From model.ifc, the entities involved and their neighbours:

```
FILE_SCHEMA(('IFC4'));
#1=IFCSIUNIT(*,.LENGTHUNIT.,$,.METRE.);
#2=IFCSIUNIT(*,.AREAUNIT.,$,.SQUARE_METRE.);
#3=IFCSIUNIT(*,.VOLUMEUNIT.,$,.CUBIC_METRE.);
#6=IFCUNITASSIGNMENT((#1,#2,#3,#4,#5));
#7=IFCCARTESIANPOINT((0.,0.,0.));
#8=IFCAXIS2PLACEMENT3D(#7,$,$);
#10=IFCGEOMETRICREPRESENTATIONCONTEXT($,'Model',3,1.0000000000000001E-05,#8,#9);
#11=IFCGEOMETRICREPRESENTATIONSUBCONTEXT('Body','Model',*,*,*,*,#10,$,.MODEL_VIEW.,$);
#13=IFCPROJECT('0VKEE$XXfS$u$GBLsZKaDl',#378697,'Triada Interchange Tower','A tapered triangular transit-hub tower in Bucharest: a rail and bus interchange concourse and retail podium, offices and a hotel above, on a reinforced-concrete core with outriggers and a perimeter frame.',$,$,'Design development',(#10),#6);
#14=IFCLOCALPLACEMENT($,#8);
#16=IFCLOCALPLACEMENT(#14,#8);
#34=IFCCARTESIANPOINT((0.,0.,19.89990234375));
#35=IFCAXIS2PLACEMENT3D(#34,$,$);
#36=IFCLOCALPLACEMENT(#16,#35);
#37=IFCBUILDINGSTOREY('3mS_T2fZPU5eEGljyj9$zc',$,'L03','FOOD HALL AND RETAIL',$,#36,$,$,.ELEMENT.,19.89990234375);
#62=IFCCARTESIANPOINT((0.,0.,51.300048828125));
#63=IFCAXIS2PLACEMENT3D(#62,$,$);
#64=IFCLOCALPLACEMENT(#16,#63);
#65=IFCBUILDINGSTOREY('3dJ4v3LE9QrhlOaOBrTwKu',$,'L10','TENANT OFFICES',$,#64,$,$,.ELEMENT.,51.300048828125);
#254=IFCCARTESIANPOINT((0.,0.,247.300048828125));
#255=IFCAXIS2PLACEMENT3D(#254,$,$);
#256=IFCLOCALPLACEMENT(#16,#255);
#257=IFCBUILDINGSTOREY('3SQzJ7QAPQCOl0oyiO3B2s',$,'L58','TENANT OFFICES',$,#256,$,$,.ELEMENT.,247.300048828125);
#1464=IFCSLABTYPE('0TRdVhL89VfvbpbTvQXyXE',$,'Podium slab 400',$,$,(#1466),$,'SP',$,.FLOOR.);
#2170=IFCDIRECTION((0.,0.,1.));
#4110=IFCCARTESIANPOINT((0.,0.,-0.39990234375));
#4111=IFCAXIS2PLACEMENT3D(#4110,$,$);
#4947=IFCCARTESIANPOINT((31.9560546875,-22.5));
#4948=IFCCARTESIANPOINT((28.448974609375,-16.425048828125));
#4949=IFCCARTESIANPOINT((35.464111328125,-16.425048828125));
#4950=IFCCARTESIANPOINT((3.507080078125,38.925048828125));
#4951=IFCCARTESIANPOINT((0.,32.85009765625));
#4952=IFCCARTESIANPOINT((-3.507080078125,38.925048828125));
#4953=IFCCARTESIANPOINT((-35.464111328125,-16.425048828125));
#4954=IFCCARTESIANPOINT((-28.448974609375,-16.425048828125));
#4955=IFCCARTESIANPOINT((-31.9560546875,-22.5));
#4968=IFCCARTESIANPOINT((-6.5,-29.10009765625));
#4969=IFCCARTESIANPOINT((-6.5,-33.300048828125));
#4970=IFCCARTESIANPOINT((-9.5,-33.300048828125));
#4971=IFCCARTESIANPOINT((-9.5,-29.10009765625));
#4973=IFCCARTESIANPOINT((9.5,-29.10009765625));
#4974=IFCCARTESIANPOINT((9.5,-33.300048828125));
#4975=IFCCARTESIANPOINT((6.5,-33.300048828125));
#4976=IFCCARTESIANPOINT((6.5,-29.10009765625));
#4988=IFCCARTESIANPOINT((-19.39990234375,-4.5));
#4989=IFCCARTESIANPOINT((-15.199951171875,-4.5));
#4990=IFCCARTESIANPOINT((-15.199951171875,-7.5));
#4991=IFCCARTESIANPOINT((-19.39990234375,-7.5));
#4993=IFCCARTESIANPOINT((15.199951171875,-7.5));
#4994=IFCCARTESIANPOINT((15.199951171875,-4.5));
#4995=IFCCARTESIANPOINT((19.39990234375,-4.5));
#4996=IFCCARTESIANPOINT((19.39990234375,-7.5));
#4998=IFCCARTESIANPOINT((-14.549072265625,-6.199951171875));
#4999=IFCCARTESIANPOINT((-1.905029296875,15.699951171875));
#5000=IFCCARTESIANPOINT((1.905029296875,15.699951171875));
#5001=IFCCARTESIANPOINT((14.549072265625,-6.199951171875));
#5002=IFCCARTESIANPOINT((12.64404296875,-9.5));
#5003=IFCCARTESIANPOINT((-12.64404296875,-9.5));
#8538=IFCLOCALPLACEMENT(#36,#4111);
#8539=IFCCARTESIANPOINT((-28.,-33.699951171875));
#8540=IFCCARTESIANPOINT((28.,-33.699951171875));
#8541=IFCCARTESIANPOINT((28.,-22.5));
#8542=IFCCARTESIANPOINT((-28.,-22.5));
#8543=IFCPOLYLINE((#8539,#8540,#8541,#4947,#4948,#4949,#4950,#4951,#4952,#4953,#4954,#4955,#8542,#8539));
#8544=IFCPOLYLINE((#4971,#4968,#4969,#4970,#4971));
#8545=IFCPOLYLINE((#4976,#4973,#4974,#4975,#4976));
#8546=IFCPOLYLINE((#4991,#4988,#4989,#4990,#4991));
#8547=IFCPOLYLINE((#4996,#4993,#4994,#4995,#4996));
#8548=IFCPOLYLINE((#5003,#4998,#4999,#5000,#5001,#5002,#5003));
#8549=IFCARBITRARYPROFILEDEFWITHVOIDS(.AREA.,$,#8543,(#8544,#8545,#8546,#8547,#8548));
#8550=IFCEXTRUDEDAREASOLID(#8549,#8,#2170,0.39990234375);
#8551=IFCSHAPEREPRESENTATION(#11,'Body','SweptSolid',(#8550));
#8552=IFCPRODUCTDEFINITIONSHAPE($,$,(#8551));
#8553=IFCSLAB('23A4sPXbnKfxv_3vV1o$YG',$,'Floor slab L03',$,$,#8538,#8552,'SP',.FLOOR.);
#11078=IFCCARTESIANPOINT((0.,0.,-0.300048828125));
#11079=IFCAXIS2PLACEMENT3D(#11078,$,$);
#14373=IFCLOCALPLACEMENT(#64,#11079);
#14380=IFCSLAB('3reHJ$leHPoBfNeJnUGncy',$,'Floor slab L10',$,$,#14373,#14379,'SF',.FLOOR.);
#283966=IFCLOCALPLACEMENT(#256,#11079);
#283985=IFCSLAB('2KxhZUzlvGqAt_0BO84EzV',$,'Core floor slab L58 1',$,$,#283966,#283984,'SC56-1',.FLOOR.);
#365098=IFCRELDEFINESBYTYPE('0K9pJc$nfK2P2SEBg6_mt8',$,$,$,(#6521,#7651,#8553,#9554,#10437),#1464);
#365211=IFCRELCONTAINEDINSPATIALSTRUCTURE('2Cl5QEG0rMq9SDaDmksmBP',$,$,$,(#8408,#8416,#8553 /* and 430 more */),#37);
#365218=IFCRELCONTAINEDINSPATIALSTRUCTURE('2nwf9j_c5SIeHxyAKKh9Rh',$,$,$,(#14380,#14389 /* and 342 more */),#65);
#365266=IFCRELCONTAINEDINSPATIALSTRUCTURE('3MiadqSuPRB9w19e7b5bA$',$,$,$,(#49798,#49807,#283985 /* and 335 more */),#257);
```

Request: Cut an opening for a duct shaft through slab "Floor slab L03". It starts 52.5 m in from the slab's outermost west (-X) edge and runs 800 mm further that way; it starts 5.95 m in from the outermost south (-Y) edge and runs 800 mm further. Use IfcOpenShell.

```python
import numpy as np
import ifcopenshell
import ifcopenshell.api.feature
import ifcopenshell.api.geometry
import ifcopenshell.api.root
import ifcopenshell.geom
import ifcopenshell.util.placement
import ifcopenshell.util.representation
import ifcopenshell.util.shape
import ifcopenshell.util.unit

model = ifcopenshell.open("model.ifc")
unit_scale = ifcopenshell.util.unit.calculate_unit_scale(model)
settings = ifcopenshell.geom.settings()


def volume(element):
    """Net volume in cubic metres, openings subtracted."""
    shape = ifcopenshell.geom.create_shape(settings, element)
    return ifcopenshell.util.shape.get_volume(shape.geometry)


slab = model.by_guid("23A4sPXbnKfxv_3vV1o$YG")
before = volume(slab)

# Extent in the slab's own axes, in metres. The edges named are its -X and -Y sides.
slab_shape = ifcopenshell.geom.create_shape(settings, slab)
vertices = ifcopenshell.util.shape.get_vertices(slab_shape.geometry)
x_min, y_min, bottom = vertices.min(axis=0)
top = vertices[:, 2].max()

opening = ifcopenshell.api.root.create_entity(model, ifc_class="IfcOpeningElement", name="Duct shaft opening", predefined_type="OPENING")
context = ifcopenshell.util.representation.get_context(model, "Model", "Body", "MODEL_VIEW")
width, depth = 0.8, 0.8
outline = [(0.0, 0.0), (width, 0.0), (width, depth), (0.0, depth), (0.0, 0.0)]
# Overshoot both faces by 50 mm so the cut is clean.
shape = ifcopenshell.api.geometry.add_slab_representation(
    model, context=context, depth=top - bottom + 0.1, polyline=outline
)
ifcopenshell.api.geometry.assign_representation(model, product=opening, representation=shape)

matrix = ifcopenshell.util.placement.get_local_placement(slab.ObjectPlacement)
matrix[:, 3] = matrix @ np.append(np.array([x_min + 52.5, y_min + 5.95, bottom - 0.05]) / unit_scale, 1.0)
ifcopenshell.api.geometry.edit_object_placement(model, product=opening, matrix=matrix, is_si=False)
ifcopenshell.api.feature.add_feature(model, feature=opening, element=slab)

after = volume(slab)

print(f"slab volume {before:.3f} -> {after:.3f} m3")

model.write("model_v2.ifc")
```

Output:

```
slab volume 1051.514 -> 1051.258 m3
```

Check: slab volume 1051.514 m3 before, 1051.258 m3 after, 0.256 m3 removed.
